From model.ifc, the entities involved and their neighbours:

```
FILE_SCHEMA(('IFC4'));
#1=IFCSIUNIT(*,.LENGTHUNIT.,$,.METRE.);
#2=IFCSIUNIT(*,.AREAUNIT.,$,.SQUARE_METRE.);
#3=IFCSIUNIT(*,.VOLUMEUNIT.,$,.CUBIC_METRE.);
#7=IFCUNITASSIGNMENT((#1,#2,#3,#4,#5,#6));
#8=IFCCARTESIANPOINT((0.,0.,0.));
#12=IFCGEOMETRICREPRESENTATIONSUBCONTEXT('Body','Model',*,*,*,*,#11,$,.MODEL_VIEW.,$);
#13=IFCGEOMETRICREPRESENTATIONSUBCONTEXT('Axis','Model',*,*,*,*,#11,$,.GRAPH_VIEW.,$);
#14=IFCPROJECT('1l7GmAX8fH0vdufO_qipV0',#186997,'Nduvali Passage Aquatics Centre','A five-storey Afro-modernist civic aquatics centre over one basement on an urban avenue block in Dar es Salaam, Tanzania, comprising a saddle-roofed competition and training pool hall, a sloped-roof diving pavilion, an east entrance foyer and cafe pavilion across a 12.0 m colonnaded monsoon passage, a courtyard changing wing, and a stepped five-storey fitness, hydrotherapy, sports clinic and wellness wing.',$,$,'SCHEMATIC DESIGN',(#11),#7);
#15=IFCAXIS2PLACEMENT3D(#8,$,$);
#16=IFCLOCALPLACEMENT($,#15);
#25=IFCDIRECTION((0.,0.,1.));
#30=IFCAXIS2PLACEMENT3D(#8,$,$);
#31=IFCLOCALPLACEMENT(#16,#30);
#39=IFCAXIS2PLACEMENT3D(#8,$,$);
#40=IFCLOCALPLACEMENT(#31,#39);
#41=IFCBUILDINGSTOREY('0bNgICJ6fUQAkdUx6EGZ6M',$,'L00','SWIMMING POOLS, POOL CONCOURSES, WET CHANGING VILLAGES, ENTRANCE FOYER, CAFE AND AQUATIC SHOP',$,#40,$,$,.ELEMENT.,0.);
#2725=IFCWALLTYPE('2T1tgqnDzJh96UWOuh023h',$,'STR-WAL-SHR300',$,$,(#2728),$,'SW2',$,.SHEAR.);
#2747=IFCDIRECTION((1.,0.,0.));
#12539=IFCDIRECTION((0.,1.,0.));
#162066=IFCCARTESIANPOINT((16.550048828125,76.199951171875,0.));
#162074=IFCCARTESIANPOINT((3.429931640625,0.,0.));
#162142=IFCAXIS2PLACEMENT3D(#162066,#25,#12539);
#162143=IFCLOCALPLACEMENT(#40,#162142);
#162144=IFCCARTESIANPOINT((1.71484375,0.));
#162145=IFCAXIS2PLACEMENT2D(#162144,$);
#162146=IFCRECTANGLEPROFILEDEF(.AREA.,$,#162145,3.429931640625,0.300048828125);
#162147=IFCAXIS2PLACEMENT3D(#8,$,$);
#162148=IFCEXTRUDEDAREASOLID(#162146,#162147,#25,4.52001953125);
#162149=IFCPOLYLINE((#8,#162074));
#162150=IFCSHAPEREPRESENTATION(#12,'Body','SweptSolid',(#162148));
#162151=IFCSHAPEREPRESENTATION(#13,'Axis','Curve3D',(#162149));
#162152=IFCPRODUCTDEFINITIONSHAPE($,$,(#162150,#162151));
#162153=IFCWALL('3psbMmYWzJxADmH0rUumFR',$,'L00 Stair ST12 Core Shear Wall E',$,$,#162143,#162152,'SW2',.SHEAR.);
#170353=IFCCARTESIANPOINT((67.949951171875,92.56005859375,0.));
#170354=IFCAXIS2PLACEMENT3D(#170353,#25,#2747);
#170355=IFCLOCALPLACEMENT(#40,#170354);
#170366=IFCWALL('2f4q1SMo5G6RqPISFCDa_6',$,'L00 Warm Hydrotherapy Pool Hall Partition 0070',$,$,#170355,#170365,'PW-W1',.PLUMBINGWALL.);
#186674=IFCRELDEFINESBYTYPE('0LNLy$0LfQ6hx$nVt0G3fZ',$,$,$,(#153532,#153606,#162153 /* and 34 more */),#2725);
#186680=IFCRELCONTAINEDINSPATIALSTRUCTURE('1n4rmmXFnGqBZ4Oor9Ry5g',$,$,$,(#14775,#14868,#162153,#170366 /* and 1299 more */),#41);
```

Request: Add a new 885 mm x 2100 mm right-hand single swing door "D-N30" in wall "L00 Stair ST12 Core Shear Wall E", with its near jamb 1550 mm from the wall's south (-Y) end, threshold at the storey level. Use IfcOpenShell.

```python
import numpy as np
import ifcopenshell
import ifcopenshell.api.feature
import ifcopenshell.api.geometry
import ifcopenshell.api.root
import ifcopenshell.api.spatial
import ifcopenshell.geom
import ifcopenshell.util.element
import ifcopenshell.util.placement
import ifcopenshell.util.representation
import ifcopenshell.util.shape
import ifcopenshell.util.unit

model = ifcopenshell.open("model.ifc")
unit_scale = ifcopenshell.util.unit.calculate_unit_scale(model)
settings = ifcopenshell.geom.settings()


def volume(element):
    """Net volume in cubic metres, openings subtracted."""
    shape = ifcopenshell.geom.create_shape(settings, element)
    return ifcopenshell.util.shape.get_volume(shape.geometry)


wall = model.by_guid("3psbMmYWzJxADmH0rUumFR")
storey = ifcopenshell.util.element.get_container(wall, ifc_class="IfcBuildingStorey")
context = ifcopenshell.util.representation.get_context(model, "Model", "Body", "MODEL_VIEW")
before = volume(wall)

width, height, from_end, sill = 0.885, 2.1, 1.55, 0.0  # metres

# The wall runs along its own X axis, and the end named is its -X end.
wall_shape = ifcopenshell.geom.create_shape(settings, wall)
x, y, z = ifcopenshell.util.shape.get_vertices(wall_shape.geometry).T
start = x.min() + from_end
face, thickness = float(y.min()), float(y.max() - y.min())
wall_matrix = ifcopenshell.util.placement.get_local_placement(wall.ObjectPlacement)
level = ifcopenshell.util.placement.get_local_placement(storey.ObjectPlacement)[2, 3]


def in_wall(x, y):
    """Placement at x, y metres in the wall's axes, at sill height."""
    matrix = wall_matrix.copy()
    matrix[:, 3] = wall_matrix @ np.array([x / unit_scale, y / unit_scale, 0.0, 1.0])
    matrix[2, 3] = level + sill / unit_scale
    return matrix


# Opening: a box that overshoots both wall faces by 50 mm.
opening = ifcopenshell.api.root.create_entity(model, ifc_class="IfcOpeningElement", predefined_type="OPENING")
box = ifcopenshell.api.geometry.add_wall_representation(
    model, context=context, length=width, height=height, thickness=thickness + 0.1
)
ifcopenshell.api.geometry.assign_representation(model, product=opening, representation=box)
ifcopenshell.api.geometry.edit_object_placement(model, product=opening, matrix=in_wall(start, face - 0.05), is_si=False)
ifcopenshell.api.feature.add_feature(model, feature=opening, element=wall)

door = ifcopenshell.api.root.create_entity(model, ifc_class="IfcDoor", name="D-N30", predefined_type="DOOR")
door.OverallWidth, door.OverallHeight = width / unit_scale, height / unit_scale
door.OperationType = "SINGLE_SWING_RIGHT"
body = ifcopenshell.api.geometry.add_door_representation(
    model,
    context=context,
    overall_width=door.OverallWidth,
    overall_height=door.OverallHeight,
    operation_type="SINGLE_SWING_RIGHT",
    lining_properties={"LiningDepth": thickness / unit_scale, "ThresholdDepth": thickness / unit_scale},
)
ifcopenshell.api.geometry.assign_representation(model, product=door, representation=body)
ifcopenshell.api.spatial.assign_container(model, products=[door], relating_structure=storey)
ifcopenshell.api.feature.add_filling(model, opening=opening, element=door)

# The lining spans the wall, so the door starts at the wall face.
ifcopenshell.api.geometry.edit_object_placement(model, product=door, matrix=in_wall(start, face), is_si=False)

after = volume(wall)

print(f"wall volume {before:.3f} -> {after:.3f} m3")

model.write("model_edited.ifc")
```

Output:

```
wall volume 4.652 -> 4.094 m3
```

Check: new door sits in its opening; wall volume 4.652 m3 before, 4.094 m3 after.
